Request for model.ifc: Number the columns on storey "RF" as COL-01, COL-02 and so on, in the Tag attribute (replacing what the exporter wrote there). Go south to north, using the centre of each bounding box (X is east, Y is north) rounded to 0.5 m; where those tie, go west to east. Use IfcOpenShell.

First a look at what the model holds.

```python
import ifcopenshell
import ifcopenshell.util.element
import ifcopenshell.util.placement

model = ifcopenshell.open("model.ifc")
print(model.schema)
storey = next(s for s in model.by_type("IfcBuildingStorey") if s.Name == "RF")
columns = [e for e in ifcopenshell.util.element.get_decomposition(storey) if e.is_a("IfcColumn")]
for e in sorted(columns, key=lambda e: e.id()):
    origin = ifcopenshell.util.placement.get_local_placement(e.ObjectPlacement)[:3, 3]
    print(e.id(), e.Tag, e.Name, origin.round(2) + 0.0, sep=" | ")
```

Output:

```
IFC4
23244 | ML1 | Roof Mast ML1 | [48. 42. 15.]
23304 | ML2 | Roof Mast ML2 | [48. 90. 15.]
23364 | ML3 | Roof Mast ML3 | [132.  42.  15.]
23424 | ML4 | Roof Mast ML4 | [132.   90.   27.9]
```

```python
import ifcopenshell
import ifcopenshell.geom
import ifcopenshell.util.element
import ifcopenshell.util.shape

model = ifcopenshell.open("model.ifc")
settings = ifcopenshell.geom.settings()
settings.set("use-world-coords", True)


def centre(element):
    shape = ifcopenshell.geom.create_shape(settings, element)
    return ifcopenshell.util.shape.get_bbox_centroid(shape.geometry)


storey = next(s for s in model.by_type("IfcBuildingStorey") if s.Name == "RF")
columns = [e for e in ifcopenshell.util.element.get_decomposition(storey) if e.is_a("IfcColumn")]

# Insertion points can sit at a corner or the storey origin, so sort by the geometry (in metres).
centres = {e: centre(e) for e in columns}
columns.sort(key=lambda e: (round(centres[e][1] / 0.5), centres[e][0]))

for i, e in enumerate(columns, start=1):
    number = f"COL-{i:02d}"
    e.Tag = number
    print(e.id(), number)

model.write("model_rev.ifc")
```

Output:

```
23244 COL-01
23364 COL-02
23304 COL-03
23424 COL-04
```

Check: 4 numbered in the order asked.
